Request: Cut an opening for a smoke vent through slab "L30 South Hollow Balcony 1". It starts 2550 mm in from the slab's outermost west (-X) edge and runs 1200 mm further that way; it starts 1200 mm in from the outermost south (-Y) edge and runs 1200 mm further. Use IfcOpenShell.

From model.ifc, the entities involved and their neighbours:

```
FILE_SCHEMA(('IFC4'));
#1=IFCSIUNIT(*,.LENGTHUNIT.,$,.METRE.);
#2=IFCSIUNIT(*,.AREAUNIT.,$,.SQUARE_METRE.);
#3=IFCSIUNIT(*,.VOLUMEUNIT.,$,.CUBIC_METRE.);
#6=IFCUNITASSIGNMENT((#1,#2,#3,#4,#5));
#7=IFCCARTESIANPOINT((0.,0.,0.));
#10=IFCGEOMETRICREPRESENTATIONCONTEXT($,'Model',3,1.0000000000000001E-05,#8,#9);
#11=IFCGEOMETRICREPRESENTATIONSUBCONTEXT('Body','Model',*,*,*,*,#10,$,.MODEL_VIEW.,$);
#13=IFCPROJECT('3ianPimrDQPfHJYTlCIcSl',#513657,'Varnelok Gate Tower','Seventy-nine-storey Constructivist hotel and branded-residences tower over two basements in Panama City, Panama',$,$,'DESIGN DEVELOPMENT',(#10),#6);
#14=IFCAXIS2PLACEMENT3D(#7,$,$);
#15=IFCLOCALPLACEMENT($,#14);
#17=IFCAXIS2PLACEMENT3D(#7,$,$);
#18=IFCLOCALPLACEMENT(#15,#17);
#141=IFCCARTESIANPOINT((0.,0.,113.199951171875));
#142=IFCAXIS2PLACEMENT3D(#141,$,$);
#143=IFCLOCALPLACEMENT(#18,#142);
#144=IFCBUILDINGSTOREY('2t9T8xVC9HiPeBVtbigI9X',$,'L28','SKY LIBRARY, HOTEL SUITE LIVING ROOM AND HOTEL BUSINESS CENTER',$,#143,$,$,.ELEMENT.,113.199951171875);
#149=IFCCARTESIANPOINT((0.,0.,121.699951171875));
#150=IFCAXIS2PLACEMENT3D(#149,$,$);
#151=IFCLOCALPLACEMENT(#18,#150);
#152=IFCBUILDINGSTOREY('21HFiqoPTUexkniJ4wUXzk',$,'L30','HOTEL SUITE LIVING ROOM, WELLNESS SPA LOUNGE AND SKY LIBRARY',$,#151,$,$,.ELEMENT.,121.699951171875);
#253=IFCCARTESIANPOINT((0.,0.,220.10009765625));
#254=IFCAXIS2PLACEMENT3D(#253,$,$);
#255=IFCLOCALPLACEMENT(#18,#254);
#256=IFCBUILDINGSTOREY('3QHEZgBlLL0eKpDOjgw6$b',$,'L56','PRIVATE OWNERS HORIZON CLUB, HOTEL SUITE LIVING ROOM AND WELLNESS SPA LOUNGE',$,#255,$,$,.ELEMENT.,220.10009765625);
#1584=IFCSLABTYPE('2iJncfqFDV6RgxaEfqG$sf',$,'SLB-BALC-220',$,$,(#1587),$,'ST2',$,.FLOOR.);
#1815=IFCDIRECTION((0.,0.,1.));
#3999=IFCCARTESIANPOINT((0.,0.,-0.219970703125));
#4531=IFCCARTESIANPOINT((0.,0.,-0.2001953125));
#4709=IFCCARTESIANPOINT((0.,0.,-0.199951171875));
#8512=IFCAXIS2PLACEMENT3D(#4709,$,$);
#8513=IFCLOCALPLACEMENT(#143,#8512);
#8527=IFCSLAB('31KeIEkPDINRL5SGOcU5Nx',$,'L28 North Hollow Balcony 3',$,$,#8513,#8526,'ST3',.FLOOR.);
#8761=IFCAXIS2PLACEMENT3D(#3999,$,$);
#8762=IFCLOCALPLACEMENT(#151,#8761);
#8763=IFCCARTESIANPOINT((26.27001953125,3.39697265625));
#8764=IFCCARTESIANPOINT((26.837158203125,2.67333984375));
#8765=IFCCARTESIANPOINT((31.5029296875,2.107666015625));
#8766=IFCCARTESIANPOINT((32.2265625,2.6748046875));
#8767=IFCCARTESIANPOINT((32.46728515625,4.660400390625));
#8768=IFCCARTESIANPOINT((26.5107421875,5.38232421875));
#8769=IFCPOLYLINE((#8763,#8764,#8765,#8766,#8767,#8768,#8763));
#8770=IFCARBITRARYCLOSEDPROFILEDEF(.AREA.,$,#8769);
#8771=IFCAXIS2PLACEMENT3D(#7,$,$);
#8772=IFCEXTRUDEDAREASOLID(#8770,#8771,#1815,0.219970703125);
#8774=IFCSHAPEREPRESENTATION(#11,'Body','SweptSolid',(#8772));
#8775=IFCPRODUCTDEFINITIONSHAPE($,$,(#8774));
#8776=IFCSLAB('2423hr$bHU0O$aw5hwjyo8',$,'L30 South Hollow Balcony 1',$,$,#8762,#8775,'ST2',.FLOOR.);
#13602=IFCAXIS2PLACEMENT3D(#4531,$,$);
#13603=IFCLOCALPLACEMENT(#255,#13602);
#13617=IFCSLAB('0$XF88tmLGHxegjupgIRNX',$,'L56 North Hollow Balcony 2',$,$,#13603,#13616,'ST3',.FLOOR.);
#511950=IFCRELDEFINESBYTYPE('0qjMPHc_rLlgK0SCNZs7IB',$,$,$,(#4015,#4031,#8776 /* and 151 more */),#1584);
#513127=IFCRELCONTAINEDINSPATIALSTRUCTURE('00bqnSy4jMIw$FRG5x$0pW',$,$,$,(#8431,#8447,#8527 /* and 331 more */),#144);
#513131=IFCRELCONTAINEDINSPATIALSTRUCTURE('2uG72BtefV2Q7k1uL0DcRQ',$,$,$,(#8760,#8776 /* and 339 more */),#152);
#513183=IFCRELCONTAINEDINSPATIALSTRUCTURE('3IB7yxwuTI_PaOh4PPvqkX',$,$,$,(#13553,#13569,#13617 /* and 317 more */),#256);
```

```python
import numpy as np
import ifcopenshell
import ifcopenshell.api.feature
import ifcopenshell.api.geometry
import ifcopenshell.api.root
import ifcopenshell.geom
import ifcopenshell.util.placement
import ifcopenshell.util.representation
import ifcopenshell.util.shape
import ifcopenshell.util.unit

model = ifcopenshell.open("model.ifc")
unit_scale = ifcopenshell.util.unit.calculate_unit_scale(model)
settings = ifcopenshell.geom.settings()


def volume(element):
    """Net volume in cubic metres, openings subtracted."""
    shape = ifcopenshell.geom.create_shape(settings, element)
    return ifcopenshell.util.shape.get_volume(shape.geometry)


slab = model.by_guid("2423hr$bHU0O$aw5hwjyo8")
before = volume(slab)

# Extent in the slab's own axes, in metres. The edges named are its -X and -Y sides.
slab_shape = ifcopenshell.geom.create_shape(settings, slab)
vertices = ifcopenshell.util.shape.get_vertices(slab_shape.geometry)
x_min, y_min, bottom = vertices.min(axis=0)
top = vertices[:, 2].max()

opening = ifcopenshell.api.root.create_entity(model, ifc_class="IfcOpeningElement", name="Smoke vent opening", predefined_type="OPENING")
context = ifcopenshell.util.representation.get_context(model, "Model", "Body", "MODEL_VIEW")
width, depth = 1.2, 1.2
outline = [(0.0, 0.0), (width, 0.0), (width, depth), (0.0, depth), (0.0, 0.0)]
# Overshoot both faces by 50 mm so the cut is clean.
shape = ifcopenshell.api.geometry.add_slab_representation(
    model, context=context, depth=top - bottom + 0.1, polyline=outline
)
ifcopenshell.api.geometry.assign_representation(model, product=opening, representation=shape)

matrix = ifcopenshell.util.placement.get_local_placement(slab.ObjectPlacement)
matrix[:, 3] = matrix @ np.append(np.array([x_min + 2.55, y_min + 1.2, bottom - 0.05]) / unit_scale, 1.0)
ifcopenshell.api.geometry.edit_object_placement(model, product=opening, matrix=matrix, is_si=False)
ifcopenshell.api.feature.add_feature(model, feature=opening, element=slab)

after = volume(slab)

print(f"slab volume {before:.3f} -> {after:.3f} m3")

model.write("model_rev.ifc")
```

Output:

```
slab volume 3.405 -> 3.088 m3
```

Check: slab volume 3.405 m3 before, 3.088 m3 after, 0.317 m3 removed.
